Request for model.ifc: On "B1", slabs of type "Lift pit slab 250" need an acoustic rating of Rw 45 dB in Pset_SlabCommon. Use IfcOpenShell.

First a look at what the model holds.

```python
import ifcopenshell
import ifcopenshell.util.element

model = ifcopenshell.open("model.ifc")
print(model.schema)
storey = next(s for s in model.by_type("IfcBuildingStorey") if s.Name == "B1")
slabs = [e for e in ifcopenshell.util.element.get_decomposition(storey) if e.is_a("IfcSlab")]
seen = {}
for e in slabs:
    element_type = ifcopenshell.util.element.get_type(e)
    key = (element_type.Name if element_type != e and element_type else None, ifcopenshell.util.element.get_pset(e, "Pset_SlabCommon", "AcousticRating"))
    seen[key] = seen.get(key, 0) + 1
for (name, value), count in sorted(seen.items(), key=str):
    print(count, "x", name, "|", value)
```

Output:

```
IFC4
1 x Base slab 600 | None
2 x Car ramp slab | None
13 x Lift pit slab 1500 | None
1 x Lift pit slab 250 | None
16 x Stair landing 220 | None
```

```python
import ifcopenshell
import ifcopenshell.api.pset
import ifcopenshell.util.element

model = ifcopenshell.open("model.ifc")

storey = next(s for s in model.by_type("IfcBuildingStorey") if s.Name == "B1")
slabs = [e for e in ifcopenshell.util.element.get_decomposition(storey) if e.is_a("IfcSlab")]

count = 0
for e in slabs:
    element_type = ifcopenshell.util.element.get_type(e)
    if element_type in (None, e) or element_type.Name != "Lift pit slab 250":
        continue
    # add_pset returns the element's existing set when there is one.
    pset = ifcopenshell.api.pset.add_pset(model, product=e, name="Pset_SlabCommon")
    ifcopenshell.api.pset.edit_pset(model, pset=pset, properties={"AcousticRating": "Rw 45 dB"})
    count += 1

print(count, "slabs updated")

model.write("model_v2.ifc")
```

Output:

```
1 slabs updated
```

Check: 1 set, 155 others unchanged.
